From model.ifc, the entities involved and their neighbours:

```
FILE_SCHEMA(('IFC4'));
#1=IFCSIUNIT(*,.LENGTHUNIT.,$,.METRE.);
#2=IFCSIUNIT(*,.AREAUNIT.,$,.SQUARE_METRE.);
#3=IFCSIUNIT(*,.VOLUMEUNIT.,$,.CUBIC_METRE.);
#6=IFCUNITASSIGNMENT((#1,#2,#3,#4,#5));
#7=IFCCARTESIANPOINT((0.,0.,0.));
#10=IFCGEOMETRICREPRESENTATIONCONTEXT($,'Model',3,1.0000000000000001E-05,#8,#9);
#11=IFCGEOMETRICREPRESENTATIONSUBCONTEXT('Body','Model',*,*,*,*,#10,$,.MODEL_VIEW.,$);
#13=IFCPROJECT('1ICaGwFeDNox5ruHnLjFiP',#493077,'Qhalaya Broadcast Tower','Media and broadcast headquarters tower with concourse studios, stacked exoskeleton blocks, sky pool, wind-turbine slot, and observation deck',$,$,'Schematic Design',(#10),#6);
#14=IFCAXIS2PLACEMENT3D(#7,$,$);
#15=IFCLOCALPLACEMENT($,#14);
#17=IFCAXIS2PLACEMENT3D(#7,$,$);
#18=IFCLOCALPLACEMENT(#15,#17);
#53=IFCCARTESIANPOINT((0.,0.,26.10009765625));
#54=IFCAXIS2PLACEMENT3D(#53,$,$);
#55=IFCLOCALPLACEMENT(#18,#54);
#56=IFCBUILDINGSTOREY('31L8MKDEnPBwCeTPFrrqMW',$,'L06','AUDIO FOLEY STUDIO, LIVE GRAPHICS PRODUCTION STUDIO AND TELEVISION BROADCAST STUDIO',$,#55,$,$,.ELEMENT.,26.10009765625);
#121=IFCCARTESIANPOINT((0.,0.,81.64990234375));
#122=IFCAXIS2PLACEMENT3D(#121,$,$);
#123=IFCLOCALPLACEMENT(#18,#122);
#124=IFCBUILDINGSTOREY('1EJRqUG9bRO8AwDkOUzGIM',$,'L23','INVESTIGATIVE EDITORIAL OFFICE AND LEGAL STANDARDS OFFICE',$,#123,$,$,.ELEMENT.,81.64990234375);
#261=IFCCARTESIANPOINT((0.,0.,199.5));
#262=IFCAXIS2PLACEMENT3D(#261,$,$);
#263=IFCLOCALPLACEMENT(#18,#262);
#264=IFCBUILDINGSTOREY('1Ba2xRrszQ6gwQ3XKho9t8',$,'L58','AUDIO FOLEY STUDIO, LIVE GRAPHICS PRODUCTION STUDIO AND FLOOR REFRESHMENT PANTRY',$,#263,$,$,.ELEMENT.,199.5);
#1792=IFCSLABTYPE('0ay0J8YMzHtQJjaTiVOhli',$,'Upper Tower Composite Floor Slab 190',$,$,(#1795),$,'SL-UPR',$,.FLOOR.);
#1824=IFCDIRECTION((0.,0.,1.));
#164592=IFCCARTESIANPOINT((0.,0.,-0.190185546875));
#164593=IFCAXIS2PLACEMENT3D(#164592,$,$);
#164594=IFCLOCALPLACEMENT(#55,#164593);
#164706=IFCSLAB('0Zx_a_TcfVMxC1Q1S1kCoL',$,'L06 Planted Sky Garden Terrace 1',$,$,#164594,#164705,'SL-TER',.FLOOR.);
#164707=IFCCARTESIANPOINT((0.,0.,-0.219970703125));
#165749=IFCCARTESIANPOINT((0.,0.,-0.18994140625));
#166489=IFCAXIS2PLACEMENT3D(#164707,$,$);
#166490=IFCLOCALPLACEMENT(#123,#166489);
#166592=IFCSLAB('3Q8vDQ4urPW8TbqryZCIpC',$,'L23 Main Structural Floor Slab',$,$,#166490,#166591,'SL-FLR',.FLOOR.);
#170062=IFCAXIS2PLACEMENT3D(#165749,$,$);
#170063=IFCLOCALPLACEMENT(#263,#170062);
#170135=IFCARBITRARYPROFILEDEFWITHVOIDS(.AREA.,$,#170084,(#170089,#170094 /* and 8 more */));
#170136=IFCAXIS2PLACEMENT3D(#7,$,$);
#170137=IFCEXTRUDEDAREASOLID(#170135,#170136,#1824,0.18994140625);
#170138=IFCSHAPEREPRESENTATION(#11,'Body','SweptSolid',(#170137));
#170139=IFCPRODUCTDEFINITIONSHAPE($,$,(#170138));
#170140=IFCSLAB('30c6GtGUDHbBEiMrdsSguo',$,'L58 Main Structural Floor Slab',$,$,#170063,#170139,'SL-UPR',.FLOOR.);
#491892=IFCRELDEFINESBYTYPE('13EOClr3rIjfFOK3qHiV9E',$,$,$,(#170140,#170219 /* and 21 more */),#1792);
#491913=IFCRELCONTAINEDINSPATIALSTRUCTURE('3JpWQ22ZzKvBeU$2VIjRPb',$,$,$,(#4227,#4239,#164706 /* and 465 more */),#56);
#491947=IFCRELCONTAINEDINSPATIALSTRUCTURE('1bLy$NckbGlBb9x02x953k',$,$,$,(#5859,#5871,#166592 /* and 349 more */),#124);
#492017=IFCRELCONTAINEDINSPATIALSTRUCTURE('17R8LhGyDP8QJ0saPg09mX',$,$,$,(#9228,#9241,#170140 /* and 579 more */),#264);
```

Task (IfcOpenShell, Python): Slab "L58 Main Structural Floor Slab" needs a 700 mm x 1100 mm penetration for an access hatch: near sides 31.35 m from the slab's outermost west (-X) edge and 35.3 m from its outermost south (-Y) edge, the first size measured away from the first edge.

```python
import numpy as np
import ifcopenshell
import ifcopenshell.api.feature
import ifcopenshell.api.geometry
import ifcopenshell.api.root
import ifcopenshell.geom
import ifcopenshell.util.placement
import ifcopenshell.util.representation
import ifcopenshell.util.shape
import ifcopenshell.util.unit

model = ifcopenshell.open("model.ifc")
unit_scale = ifcopenshell.util.unit.calculate_unit_scale(model)
settings = ifcopenshell.geom.settings()


def volume(element):
    """Net volume in cubic metres, openings subtracted."""
    shape = ifcopenshell.geom.create_shape(settings, element)
    return ifcopenshell.util.shape.get_volume(shape.geometry)


slab = model.by_guid("30c6GtGUDHbBEiMrdsSguo")
before = volume(slab)

# Extent in the slab's own axes, in metres. The edges named are its -X and -Y sides.
slab_shape = ifcopenshell.geom.create_shape(settings, slab)
vertices = ifcopenshell.util.shape.get_vertices(slab_shape.geometry)
x_min, y_min, bottom = vertices.min(axis=0)
top = vertices[:, 2].max()

opening = ifcopenshell.api.root.create_entity(model, ifc_class="IfcOpeningElement", name="Access hatch opening", predefined_type="OPENING")
context = ifcopenshell.util.representation.get_context(model, "Model", "Body", "MODEL_VIEW")
width, depth = 0.7, 1.1
outline = [(0.0, 0.0), (width, 0.0), (width, depth), (0.0, depth), (0.0, 0.0)]
# Overshoot both faces by 50 mm so the cut is clean.
shape = ifcopenshell.api.geometry.add_slab_representation(
    model, context=context, depth=top - bottom + 0.1, polyline=outline
)
ifcopenshell.api.geometry.assign_representation(model, product=opening, representation=shape)

matrix = ifcopenshell.util.placement.get_local_placement(slab.ObjectPlacement)
matrix[:, 3] = matrix @ np.append(np.array([x_min + 31.35, y_min + 35.3, bottom - 0.05]) / unit_scale, 1.0)
ifcopenshell.api.geometry.edit_object_placement(model, product=opening, matrix=matrix, is_si=False)
ifcopenshell.api.feature.add_feature(model, feature=opening, element=slab)

after = volume(slab)

print(f"slab volume {before:.3f} -> {after:.3f} m3")

model.write("model_v2.ifc")
```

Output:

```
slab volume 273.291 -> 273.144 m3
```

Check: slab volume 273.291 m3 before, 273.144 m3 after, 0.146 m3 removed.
